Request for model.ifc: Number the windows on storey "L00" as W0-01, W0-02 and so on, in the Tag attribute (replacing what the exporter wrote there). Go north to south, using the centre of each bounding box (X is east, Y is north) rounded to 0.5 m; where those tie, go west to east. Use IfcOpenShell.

First a look at what the model holds.

```python
import ifcopenshell
import ifcopenshell.util.element
import ifcopenshell.util.placement

model = ifcopenshell.open("model.ifc")
print(model.schema)
storey = next(s for s in model.by_type("IfcBuildingStorey") if s.Name == "L00")
windows = [e for e in ifcopenshell.util.element.get_decomposition(storey) if e.is_a("IfcWindow")]
for e in sorted(windows, key=lambda e: e.id()):
    origin = ifcopenshell.util.placement.get_local_placement(e.ObjectPlacement)[:3, 3]
    print(e.id(), e.Tag, e.Name, origin.round(2) + 0.0, sep=" | ")
```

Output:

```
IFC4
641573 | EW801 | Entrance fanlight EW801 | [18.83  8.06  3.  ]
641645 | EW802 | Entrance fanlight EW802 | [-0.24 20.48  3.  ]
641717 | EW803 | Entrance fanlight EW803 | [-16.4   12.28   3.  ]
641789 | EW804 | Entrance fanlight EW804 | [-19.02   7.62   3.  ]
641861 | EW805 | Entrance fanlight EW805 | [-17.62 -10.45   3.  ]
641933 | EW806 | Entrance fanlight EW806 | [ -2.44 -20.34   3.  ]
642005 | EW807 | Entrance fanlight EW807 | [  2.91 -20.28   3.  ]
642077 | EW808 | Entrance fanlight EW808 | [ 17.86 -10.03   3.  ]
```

```python
import ifcopenshell
import ifcopenshell.geom
import ifcopenshell.util.element
import ifcopenshell.util.shape

model = ifcopenshell.open("model.ifc")
settings = ifcopenshell.geom.settings()
settings.set("use-world-coords", True)


def centre(element):
    shape = ifcopenshell.geom.create_shape(settings, element)
    return ifcopenshell.util.shape.get_bbox_centroid(shape.geometry)


storey = next(s for s in model.by_type("IfcBuildingStorey") if s.Name == "L00")
windows = [e for e in ifcopenshell.util.element.get_decomposition(storey) if e.is_a("IfcWindow")]

# Insertion points can sit at a corner or the storey origin, so sort by the geometry (in metres).
centres = {e: centre(e) for e in windows}
windows.sort(key=lambda e: (-round(centres[e][1] / 0.5), centres[e][0]))

for i, e in enumerate(windows, start=1):
    number = f"W0-{i:02d}"
    e.Tag = number
    print(e.id(), number)

model.write("model_rev.ifc")
```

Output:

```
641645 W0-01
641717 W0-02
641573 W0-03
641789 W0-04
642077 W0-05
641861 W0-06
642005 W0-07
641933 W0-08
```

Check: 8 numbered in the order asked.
